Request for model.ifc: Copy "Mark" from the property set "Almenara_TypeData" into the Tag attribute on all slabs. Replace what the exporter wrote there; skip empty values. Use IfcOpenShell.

First a look at what the model holds.

```python
import ifcopenshell
import ifcopenshell.util.element

model = ifcopenshell.open("model.ifc")
print(model.schema)
slabs = model.by_type("IfcSlab")
print(len(slabs), "slabs")
for e in slabs[:8]:
    source = ifcopenshell.util.element.get_pset(e, "Almenara_TypeData", "Mark")
    target = e.Tag
    print(e.id(), repr(source), repr(target), sep=" | ")
```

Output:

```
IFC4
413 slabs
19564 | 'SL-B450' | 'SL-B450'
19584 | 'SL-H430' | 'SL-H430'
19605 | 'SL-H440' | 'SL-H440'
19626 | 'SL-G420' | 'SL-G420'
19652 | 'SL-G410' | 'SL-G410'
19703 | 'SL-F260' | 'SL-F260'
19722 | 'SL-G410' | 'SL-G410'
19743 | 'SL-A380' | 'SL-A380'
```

```python
import ifcopenshell
import ifcopenshell.util.element

model = ifcopenshell.open("model.ifc")

count = 0
for e in model.by_type("IfcSlab"):
    value = ifcopenshell.util.element.get_pset(e, "Almenara_TypeData", "Mark")
    current = e.Tag
    if not value or not value.strip() or current == value:
        continue
    e.Tag = value
    count += 1

print(count, "slabs updated")

model.write("model_rev.ifc")
```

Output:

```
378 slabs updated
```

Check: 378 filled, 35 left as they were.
